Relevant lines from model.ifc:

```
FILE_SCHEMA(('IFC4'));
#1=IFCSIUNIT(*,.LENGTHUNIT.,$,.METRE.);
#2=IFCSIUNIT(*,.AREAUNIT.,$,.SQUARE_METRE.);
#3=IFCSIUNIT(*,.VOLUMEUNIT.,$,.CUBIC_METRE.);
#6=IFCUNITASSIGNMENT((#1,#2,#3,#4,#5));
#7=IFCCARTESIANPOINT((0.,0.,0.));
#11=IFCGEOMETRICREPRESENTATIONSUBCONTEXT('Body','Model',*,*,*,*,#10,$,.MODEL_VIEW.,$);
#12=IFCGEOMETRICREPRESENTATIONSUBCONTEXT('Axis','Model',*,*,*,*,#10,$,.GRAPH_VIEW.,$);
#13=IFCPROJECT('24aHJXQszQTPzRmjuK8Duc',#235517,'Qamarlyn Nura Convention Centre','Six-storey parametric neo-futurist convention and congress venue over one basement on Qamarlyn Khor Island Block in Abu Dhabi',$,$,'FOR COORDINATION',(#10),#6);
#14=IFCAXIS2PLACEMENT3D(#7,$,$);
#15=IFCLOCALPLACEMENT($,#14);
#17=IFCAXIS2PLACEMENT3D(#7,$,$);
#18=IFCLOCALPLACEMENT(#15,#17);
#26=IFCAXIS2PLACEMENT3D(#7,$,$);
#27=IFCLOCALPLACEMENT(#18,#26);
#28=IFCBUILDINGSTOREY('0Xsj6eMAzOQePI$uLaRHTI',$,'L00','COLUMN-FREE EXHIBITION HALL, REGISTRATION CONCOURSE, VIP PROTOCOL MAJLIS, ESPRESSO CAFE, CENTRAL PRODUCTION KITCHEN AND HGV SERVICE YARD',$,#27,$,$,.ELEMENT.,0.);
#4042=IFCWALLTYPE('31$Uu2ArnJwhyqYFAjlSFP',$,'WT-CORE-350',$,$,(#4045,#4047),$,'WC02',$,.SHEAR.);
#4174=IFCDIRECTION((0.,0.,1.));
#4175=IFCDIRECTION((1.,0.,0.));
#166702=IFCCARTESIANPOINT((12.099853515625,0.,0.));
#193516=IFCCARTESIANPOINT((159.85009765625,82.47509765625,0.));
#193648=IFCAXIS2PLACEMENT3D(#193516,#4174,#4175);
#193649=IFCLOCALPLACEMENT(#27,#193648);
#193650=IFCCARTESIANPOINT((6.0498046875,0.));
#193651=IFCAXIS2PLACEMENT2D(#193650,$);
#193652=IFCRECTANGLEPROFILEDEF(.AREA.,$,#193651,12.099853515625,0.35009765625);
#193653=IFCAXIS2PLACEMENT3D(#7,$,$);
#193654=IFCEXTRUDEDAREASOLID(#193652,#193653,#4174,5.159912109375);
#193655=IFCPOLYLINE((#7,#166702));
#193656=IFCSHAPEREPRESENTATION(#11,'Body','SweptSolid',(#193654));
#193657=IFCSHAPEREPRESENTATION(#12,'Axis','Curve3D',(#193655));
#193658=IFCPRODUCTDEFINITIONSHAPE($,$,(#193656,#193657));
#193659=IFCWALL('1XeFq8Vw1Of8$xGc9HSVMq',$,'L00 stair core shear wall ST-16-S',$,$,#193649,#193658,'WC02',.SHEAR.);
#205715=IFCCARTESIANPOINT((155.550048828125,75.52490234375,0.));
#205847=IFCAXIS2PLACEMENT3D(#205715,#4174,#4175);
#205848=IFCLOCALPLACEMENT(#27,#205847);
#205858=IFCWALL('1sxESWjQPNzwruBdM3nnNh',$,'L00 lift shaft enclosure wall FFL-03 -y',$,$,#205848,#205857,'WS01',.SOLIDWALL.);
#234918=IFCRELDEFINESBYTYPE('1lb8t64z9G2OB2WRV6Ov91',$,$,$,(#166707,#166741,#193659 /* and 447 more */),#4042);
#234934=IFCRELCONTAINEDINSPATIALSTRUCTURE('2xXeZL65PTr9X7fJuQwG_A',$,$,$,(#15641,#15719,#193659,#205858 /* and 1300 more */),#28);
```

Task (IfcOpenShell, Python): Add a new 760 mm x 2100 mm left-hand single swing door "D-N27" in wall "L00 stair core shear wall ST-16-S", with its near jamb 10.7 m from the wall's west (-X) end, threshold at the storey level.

```python
import numpy as np
import ifcopenshell
import ifcopenshell.api.feature
import ifcopenshell.api.geometry
import ifcopenshell.api.root
import ifcopenshell.api.spatial
import ifcopenshell.geom
import ifcopenshell.util.element
import ifcopenshell.util.placement
import ifcopenshell.util.representation
import ifcopenshell.util.shape
import ifcopenshell.util.unit

model = ifcopenshell.open("model.ifc")
unit_scale = ifcopenshell.util.unit.calculate_unit_scale(model)
settings = ifcopenshell.geom.settings()


def volume(element):
    """Net volume in cubic metres, openings subtracted."""
    shape = ifcopenshell.geom.create_shape(settings, element)
    return ifcopenshell.util.shape.get_volume(shape.geometry)


wall = model.by_id(193659)
storey = ifcopenshell.util.element.get_container(wall, ifc_class="IfcBuildingStorey")
context = ifcopenshell.util.representation.get_context(model, "Model", "Body", "MODEL_VIEW")
before = volume(wall)

width, height, from_end, sill = 0.76, 2.1, 10.7, 0.0  # metres

# The wall runs along its own X axis, and the end named is its -X end.
wall_shape = ifcopenshell.geom.create_shape(settings, wall)
x, y, z = ifcopenshell.util.shape.get_vertices(wall_shape.geometry).T
start = x.min() + from_end
face, thickness = float(y.min()), float(y.max() - y.min())
wall_matrix = ifcopenshell.util.placement.get_local_placement(wall.ObjectPlacement)
level = ifcopenshell.util.placement.get_local_placement(storey.ObjectPlacement)[2, 3]


def in_wall(x, y):
    """Placement at x, y metres in the wall's axes, at sill height."""
    matrix = wall_matrix.copy()
    matrix[:, 3] = wall_matrix @ np.array([x / unit_scale, y / unit_scale, 0.0, 1.0])
    matrix[2, 3] = level + sill / unit_scale
    return matrix


# Opening: a box that overshoots both wall faces by 50 mm.
opening = ifcopenshell.api.root.create_entity(model, ifc_class="IfcOpeningElement", predefined_type="OPENING")
box = ifcopenshell.api.geometry.add_wall_representation(
    model, context=context, length=width, height=height, thickness=thickness + 0.1
)
ifcopenshell.api.geometry.assign_representation(model, product=opening, representation=box)
ifcopenshell.api.geometry.edit_object_placement(model, product=opening, matrix=in_wall(start, face - 0.05), is_si=False)
ifcopenshell.api.feature.add_feature(model, feature=opening, element=wall)

door = ifcopenshell.api.root.create_entity(model, ifc_class="IfcDoor", name="D-N27", predefined_type="DOOR")
door.OverallWidth, door.OverallHeight = width / unit_scale, height / unit_scale
door.OperationType = "SINGLE_SWING_LEFT"
body = ifcopenshell.api.geometry.add_door_representation(
    model,
    context=context,
    overall_width=door.OverallWidth,
    overall_height=door.OverallHeight,
    operation_type="SINGLE_SWING_LEFT",
    lining_properties={"LiningDepth": thickness / unit_scale, "ThresholdDepth": thickness / unit_scale},
)
ifcopenshell.api.geometry.assign_representation(model, product=door, representation=body)
ifcopenshell.api.spatial.assign_container(model, products=[door], relating_structure=storey)
ifcopenshell.api.feature.add_filling(model, opening=opening, element=door)

# The lining spans the wall, so the door starts at the wall face.
ifcopenshell.api.geometry.edit_object_placement(model, product=door, matrix=in_wall(start, face), is_si=False)

after = volume(wall)

print(f"wall volume {before:.3f} -> {after:.3f} m3")

model.write("model_v2.ifc")
```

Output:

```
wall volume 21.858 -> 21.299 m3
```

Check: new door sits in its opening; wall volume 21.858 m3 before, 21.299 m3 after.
